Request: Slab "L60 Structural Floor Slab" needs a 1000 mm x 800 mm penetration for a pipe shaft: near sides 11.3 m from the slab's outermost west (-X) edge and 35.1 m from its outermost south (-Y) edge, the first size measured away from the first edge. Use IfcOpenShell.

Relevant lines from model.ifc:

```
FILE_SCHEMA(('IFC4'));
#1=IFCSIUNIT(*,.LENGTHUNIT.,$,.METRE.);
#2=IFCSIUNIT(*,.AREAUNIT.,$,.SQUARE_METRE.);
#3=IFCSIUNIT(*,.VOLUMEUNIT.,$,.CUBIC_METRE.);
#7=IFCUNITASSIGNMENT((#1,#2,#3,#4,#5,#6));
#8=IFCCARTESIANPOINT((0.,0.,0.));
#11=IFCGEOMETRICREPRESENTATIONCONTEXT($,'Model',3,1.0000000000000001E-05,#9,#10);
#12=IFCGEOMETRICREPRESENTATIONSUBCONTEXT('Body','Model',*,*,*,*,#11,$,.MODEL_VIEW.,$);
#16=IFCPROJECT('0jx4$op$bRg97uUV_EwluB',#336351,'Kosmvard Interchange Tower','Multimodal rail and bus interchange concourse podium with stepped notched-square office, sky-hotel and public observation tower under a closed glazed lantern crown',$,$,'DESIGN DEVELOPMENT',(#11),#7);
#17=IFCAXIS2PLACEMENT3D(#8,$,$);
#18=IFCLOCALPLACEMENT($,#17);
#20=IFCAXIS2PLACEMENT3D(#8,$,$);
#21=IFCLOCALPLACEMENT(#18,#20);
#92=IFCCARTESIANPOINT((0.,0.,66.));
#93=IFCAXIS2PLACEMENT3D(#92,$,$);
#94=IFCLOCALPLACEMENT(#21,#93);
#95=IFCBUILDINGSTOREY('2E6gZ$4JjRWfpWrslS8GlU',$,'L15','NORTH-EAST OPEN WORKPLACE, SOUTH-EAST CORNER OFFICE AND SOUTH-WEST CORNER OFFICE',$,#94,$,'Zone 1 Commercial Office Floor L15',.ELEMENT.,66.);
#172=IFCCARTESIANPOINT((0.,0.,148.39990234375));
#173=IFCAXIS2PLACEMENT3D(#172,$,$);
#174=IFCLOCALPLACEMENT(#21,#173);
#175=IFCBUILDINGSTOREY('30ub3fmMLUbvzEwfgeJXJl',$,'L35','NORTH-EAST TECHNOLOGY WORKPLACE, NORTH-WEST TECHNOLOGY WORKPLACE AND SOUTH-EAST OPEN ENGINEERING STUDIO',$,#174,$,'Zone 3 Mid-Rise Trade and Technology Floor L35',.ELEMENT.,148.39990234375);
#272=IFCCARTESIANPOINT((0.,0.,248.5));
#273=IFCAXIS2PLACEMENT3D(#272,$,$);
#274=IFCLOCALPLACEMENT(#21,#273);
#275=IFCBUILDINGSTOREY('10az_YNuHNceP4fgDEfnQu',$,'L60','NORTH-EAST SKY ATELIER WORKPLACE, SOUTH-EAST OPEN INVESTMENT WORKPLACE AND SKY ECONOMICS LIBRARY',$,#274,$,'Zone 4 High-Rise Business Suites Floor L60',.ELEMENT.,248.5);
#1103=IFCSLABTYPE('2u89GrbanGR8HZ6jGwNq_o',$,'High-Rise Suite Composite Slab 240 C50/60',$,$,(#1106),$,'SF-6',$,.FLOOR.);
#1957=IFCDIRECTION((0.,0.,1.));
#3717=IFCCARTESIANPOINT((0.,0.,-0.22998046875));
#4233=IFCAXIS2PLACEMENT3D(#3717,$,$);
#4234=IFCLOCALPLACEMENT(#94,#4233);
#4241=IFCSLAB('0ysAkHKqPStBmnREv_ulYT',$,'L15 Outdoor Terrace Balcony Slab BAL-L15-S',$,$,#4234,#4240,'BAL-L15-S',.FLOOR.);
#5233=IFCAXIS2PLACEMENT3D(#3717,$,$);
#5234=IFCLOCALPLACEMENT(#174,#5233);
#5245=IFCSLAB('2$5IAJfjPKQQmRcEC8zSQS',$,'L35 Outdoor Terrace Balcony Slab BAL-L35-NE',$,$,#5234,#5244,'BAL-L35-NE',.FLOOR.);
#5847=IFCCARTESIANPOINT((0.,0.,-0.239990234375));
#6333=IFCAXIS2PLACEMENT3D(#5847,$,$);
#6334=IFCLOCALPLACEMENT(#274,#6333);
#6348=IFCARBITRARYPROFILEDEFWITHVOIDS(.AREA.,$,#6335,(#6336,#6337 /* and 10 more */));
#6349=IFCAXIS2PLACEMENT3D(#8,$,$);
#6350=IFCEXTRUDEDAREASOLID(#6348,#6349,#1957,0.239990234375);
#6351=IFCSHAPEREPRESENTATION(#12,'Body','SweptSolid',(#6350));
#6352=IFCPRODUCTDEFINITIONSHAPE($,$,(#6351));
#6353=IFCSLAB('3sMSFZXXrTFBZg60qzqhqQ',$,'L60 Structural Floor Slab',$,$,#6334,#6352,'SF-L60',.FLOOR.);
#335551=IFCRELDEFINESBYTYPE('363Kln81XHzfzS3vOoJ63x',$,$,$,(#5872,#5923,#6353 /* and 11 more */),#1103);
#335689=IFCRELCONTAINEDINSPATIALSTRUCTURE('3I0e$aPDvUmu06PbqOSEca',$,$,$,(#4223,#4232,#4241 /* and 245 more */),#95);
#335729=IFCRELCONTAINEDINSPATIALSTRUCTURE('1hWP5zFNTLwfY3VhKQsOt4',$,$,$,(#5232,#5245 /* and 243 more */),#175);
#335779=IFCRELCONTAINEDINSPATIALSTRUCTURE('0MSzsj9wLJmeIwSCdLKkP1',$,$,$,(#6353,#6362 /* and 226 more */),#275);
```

```python
import numpy as np
import ifcopenshell
import ifcopenshell.api.feature
import ifcopenshell.api.geometry
import ifcopenshell.api.root
import ifcopenshell.geom
import ifcopenshell.util.placement
import ifcopenshell.util.representation
import ifcopenshell.util.shape
import ifcopenshell.util.unit

model = ifcopenshell.open("model.ifc")
unit_scale = ifcopenshell.util.unit.calculate_unit_scale(model)
settings = ifcopenshell.geom.settings()


def volume(element):
    """Net volume in cubic metres, openings subtracted."""
    shape = ifcopenshell.geom.create_shape(settings, element)
    return ifcopenshell.util.shape.get_volume(shape.geometry)


slab = model.by_guid("3sMSFZXXrTFBZg60qzqhqQ")
before = volume(slab)

# Extent in the slab's own axes, in metres. The edges named are its -X and -Y sides.
slab_shape = ifcopenshell.geom.create_shape(settings, slab)
vertices = ifcopenshell.util.shape.get_vertices(slab_shape.geometry)
x_min, y_min, bottom = vertices.min(axis=0)
top = vertices[:, 2].max()

opening = ifcopenshell.api.root.create_entity(model, ifc_class="IfcOpeningElement", name="Pipe shaft opening", predefined_type="OPENING")
context = ifcopenshell.util.representation.get_context(model, "Model", "Body", "MODEL_VIEW")
width, depth = 1, 0.8
outline = [(0.0, 0.0), (width, 0.0), (width, depth), (0.0, depth), (0.0, 0.0)]
# Overshoot both faces by 50 mm so the cut is clean.
shape = ifcopenshell.api.geometry.add_slab_representation(
    model, context=context, depth=top - bottom + 0.1, polyline=outline
)
ifcopenshell.api.geometry.assign_representation(model, product=opening, representation=shape)

matrix = ifcopenshell.util.placement.get_local_placement(slab.ObjectPlacement)
matrix[:, 3] = matrix @ np.append(np.array([x_min + 11.3, y_min + 35.1, bottom - 0.05]) / unit_scale, 1.0)
ifcopenshell.api.geometry.edit_object_placement(model, product=opening, matrix=matrix, is_si=False)
ifcopenshell.api.feature.add_feature(model, feature=opening, element=slab)

after = volume(slab)

print(f"slab volume {before:.3f} -> {after:.3f} m3")

model.write("model-out.ifc")
```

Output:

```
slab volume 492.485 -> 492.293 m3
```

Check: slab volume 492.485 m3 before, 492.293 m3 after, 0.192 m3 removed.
